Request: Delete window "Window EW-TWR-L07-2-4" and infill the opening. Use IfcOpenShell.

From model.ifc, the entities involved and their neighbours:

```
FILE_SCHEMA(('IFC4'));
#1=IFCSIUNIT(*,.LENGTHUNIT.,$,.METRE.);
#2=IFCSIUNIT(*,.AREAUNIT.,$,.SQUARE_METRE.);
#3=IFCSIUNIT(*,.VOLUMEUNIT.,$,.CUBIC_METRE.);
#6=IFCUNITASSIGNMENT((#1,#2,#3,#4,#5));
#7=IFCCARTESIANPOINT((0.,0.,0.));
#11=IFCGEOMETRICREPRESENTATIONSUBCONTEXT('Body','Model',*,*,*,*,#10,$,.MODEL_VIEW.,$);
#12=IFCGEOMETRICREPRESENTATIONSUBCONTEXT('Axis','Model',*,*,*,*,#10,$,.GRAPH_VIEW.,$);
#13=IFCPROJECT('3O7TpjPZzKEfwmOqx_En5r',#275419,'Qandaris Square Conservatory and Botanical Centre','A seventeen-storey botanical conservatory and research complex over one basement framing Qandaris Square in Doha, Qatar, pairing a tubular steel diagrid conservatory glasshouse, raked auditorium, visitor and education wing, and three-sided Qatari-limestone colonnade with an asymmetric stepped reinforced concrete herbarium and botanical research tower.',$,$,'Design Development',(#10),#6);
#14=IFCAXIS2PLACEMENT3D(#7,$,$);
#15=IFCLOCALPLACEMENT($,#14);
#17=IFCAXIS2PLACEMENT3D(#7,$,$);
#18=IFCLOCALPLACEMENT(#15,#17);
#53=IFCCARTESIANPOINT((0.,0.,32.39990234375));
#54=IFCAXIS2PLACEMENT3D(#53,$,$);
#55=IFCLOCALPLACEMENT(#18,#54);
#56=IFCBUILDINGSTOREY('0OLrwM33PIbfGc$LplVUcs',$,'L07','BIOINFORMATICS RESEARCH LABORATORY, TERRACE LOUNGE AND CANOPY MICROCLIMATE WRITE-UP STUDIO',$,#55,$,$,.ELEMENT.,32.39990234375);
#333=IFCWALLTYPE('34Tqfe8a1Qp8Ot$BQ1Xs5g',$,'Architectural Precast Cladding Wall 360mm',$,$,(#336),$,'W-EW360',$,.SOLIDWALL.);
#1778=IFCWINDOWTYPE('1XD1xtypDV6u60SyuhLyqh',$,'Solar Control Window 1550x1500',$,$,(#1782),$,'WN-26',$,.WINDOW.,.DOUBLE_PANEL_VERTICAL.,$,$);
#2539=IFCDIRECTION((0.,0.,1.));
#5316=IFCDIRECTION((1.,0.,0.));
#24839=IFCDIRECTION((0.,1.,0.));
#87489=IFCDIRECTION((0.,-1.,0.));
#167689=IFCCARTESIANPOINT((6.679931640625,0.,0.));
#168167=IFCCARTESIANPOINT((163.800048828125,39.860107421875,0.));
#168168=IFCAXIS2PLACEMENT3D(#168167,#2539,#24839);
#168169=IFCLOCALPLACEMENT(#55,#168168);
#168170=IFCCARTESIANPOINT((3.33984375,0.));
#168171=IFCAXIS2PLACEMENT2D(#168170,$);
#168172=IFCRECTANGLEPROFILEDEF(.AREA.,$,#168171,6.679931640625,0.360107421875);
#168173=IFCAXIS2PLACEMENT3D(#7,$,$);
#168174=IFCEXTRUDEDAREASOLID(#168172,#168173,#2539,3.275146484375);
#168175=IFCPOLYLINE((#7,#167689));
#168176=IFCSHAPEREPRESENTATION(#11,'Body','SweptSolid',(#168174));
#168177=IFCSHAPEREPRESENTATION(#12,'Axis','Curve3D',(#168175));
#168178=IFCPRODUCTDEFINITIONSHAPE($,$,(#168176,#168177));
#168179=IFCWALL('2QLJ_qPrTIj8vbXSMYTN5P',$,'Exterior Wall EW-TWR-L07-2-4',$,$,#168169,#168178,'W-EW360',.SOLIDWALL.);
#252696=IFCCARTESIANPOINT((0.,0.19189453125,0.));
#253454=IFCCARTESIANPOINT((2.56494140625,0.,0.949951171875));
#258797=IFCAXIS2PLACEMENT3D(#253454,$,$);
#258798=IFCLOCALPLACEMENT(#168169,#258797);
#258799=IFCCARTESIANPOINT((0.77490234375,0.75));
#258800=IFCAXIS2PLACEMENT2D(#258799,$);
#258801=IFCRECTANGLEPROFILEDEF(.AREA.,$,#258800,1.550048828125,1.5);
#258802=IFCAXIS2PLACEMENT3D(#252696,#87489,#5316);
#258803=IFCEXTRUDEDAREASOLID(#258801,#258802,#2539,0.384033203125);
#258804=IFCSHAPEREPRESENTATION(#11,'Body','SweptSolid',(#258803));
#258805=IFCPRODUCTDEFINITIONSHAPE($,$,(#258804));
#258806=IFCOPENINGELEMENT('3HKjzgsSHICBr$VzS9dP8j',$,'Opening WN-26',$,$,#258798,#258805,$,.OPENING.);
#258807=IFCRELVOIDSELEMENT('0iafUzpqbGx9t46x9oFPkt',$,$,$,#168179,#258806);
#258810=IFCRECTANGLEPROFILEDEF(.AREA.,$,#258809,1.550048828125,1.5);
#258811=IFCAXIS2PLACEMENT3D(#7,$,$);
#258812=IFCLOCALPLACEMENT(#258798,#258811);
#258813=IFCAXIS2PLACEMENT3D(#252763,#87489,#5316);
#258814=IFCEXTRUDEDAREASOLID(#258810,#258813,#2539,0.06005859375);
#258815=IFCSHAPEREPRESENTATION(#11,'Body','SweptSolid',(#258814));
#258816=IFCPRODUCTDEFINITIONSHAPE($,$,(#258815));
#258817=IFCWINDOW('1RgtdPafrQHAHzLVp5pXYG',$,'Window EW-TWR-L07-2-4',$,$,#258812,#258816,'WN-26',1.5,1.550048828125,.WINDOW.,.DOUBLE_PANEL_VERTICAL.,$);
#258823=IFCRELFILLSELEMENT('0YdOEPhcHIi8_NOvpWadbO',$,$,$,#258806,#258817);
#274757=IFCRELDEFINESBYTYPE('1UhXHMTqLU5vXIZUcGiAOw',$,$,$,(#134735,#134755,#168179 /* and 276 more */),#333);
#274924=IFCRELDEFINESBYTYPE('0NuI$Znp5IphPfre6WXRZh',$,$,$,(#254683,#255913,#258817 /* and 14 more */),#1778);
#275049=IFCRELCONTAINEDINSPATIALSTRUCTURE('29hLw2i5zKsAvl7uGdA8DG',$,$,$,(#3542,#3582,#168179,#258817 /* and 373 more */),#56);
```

```python
import ifcopenshell
import ifcopenshell.api.feature
import ifcopenshell.api.root
import ifcopenshell.geom
import ifcopenshell.util.shape

model = ifcopenshell.open("model.ifc")
settings = ifcopenshell.geom.settings()


def volume(element):
    """Net volume in cubic metres, openings subtracted."""
    shape = ifcopenshell.geom.create_shape(settings, element)
    return ifcopenshell.util.shape.get_volume(shape.geometry)


window = model.by_id(258817)
opening = window.FillsVoids[0].RelatingOpeningElement
wall = opening.VoidsElements[0].RelatingBuildingElement
before = volume(wall)

ifcopenshell.api.root.remove_product(model, product=window)
ifcopenshell.api.feature.remove_feature(model, feature=opening)

after = volume(wall)

print(f"wall volume {before:.3f} -> {after:.3f} m3")

model.write("model_rev.ifc")
```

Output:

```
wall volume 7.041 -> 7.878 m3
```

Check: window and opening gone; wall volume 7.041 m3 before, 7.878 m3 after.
